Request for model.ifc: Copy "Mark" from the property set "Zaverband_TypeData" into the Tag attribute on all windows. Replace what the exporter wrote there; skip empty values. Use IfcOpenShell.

First a look at what the model holds.

```python
import ifcopenshell
import ifcopenshell.util.element

model = ifcopenshell.open("model.ifc")
print(model.schema)
windows = model.by_type("IfcWindow")
print(len(windows), "windows")
for e in windows[:8]:
    source = ifcopenshell.util.element.get_pset(e, "Zaverband_TypeData", "Mark")
    target = e.Tag
    print(e.id(), repr(source), repr(target), sep=" | ")
```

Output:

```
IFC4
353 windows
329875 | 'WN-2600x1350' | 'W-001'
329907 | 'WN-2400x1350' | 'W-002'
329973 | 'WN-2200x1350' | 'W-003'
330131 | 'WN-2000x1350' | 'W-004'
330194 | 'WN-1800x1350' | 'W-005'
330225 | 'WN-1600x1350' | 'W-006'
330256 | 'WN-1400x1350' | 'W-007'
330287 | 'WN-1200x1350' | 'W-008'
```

```python
import ifcopenshell
import ifcopenshell.util.element

model = ifcopenshell.open("model.ifc")

count = 0
for e in model.by_type("IfcWindow"):
    value = ifcopenshell.util.element.get_pset(e, "Zaverband_TypeData", "Mark")
    current = e.Tag
    if not value or not value.strip() or current == value:
        continue
    e.Tag = value
    count += 1

print(count, "windows updated")

model.write("model_edited.ifc")
```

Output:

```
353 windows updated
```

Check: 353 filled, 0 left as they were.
